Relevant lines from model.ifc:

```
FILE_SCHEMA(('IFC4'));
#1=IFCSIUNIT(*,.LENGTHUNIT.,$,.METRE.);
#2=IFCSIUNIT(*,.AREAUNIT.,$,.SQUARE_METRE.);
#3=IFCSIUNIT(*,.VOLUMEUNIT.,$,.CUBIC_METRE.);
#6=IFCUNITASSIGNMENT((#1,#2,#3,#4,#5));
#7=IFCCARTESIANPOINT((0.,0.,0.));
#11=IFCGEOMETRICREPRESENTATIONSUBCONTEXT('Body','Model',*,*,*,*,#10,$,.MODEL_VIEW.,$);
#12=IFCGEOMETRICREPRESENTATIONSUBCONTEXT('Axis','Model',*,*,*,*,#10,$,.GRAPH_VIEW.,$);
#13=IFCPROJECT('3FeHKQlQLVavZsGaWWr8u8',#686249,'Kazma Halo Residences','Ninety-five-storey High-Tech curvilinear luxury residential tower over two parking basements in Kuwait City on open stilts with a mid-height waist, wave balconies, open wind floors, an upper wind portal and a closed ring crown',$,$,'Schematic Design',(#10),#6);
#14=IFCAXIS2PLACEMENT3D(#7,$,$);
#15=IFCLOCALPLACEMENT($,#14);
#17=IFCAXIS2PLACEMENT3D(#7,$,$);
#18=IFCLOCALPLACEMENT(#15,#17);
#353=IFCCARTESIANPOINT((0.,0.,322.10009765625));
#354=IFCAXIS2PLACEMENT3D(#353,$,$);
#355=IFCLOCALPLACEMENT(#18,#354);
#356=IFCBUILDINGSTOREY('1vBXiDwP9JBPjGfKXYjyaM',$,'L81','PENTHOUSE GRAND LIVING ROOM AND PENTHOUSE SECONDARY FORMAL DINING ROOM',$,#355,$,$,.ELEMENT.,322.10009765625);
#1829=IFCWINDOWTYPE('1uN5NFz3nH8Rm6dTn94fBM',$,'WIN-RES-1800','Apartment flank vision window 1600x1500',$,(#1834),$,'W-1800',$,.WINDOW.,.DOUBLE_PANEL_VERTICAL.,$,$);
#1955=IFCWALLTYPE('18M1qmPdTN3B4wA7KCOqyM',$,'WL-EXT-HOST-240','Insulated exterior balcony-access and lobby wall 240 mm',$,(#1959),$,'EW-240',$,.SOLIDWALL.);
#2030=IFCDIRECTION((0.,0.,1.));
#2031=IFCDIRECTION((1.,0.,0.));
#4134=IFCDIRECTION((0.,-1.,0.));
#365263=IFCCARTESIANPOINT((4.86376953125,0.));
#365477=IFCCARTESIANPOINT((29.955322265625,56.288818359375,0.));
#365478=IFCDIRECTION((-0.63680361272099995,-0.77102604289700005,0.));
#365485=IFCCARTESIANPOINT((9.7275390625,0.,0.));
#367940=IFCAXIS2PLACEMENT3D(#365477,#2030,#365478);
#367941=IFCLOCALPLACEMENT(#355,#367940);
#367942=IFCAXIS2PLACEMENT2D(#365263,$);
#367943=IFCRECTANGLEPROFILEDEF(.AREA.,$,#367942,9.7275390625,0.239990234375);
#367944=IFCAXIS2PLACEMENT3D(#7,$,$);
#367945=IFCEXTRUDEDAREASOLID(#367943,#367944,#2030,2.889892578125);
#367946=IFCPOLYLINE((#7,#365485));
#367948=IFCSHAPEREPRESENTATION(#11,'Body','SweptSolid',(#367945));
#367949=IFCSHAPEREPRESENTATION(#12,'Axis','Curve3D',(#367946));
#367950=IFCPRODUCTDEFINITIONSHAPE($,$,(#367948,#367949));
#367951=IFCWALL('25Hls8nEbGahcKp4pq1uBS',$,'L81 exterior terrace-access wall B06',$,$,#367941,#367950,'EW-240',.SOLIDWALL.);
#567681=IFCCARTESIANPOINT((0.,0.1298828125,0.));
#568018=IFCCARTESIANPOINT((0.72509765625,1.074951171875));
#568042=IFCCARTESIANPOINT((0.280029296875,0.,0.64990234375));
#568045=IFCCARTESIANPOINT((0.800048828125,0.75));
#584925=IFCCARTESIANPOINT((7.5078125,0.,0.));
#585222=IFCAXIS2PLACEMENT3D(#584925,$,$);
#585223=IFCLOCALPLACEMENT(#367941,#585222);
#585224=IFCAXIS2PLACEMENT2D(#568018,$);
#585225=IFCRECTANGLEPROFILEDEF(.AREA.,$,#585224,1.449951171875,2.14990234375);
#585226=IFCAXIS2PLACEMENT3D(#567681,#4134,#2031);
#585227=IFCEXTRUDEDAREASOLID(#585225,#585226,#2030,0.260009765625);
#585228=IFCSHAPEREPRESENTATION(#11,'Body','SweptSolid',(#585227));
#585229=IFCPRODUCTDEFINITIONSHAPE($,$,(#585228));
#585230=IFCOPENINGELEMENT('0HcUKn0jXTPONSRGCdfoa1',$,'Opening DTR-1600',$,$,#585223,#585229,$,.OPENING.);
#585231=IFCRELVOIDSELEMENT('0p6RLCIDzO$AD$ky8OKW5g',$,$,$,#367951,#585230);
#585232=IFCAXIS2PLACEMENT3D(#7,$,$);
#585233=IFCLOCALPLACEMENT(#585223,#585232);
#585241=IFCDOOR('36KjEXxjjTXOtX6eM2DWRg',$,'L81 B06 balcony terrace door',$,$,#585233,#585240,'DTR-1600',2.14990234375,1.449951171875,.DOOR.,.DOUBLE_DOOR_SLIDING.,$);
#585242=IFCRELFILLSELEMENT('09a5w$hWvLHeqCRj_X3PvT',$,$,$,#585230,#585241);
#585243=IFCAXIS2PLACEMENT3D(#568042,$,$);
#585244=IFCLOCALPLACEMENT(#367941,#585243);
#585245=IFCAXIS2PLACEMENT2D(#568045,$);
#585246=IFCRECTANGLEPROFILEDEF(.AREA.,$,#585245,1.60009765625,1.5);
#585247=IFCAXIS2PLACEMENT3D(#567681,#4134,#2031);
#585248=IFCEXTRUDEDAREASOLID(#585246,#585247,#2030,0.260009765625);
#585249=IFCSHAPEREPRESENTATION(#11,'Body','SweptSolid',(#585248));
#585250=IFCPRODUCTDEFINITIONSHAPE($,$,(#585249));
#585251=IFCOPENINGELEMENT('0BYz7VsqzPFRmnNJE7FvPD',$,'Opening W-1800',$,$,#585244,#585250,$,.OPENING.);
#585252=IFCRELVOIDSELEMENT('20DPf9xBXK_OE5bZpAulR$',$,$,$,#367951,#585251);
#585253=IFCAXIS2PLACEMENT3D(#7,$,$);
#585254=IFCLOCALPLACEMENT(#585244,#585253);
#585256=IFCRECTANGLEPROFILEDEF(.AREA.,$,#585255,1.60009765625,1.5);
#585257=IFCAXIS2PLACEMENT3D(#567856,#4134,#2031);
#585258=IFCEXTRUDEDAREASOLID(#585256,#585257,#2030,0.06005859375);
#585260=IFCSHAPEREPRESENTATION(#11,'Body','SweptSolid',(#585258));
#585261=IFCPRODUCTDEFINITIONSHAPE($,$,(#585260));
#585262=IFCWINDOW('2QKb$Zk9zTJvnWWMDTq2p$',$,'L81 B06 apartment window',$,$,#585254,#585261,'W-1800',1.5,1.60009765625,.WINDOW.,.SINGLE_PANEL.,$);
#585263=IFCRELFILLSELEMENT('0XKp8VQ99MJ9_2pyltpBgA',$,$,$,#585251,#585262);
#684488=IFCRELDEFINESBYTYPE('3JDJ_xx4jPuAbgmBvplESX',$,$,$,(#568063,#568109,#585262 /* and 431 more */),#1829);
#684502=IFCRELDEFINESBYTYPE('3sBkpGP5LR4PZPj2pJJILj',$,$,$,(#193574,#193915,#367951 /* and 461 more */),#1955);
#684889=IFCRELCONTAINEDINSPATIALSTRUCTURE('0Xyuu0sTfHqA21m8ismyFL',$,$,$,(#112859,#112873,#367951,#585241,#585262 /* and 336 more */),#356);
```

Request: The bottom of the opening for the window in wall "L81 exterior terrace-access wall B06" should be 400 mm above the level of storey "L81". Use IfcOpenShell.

```python
import numpy as np
import ifcopenshell
import ifcopenshell.api.geometry
import ifcopenshell.geom
import ifcopenshell.util.element
import ifcopenshell.util.placement
import ifcopenshell.util.shape
import ifcopenshell.util.unit

model = ifcopenshell.open("model.ifc")
unit_scale = ifcopenshell.util.unit.calculate_unit_scale(model)

window = model.by_id(585262)
opening = window.FillsVoids[0].RelatingOpeningElement
storey = ifcopenshell.util.element.get_container(window, ifc_class="IfcBuildingStorey")
level = ifcopenshell.util.placement.get_local_placement(storey.ObjectPlacement)[2, 3]

# The opening's origin need not be at the sill, so measure its lowest point.
shape = ifcopenshell.geom.create_shape(ifcopenshell.geom.settings(), opening)
bottom = ifcopenshell.util.shape.get_shape_bottom_elevation(shape, shape.geometry) / unit_scale
dz = level + 0.4 / unit_scale - bottom

shift = np.array([0.0, 0.0, dz])
# The window is placed relative to its opening, so it follows when the opening moves.
matrix = ifcopenshell.util.placement.get_local_placement(opening.ObjectPlacement)
matrix[:3, 3] += shift
ifcopenshell.api.geometry.edit_object_placement(
    model, product=opening, matrix=matrix, is_si=False, should_transform_children=True
)

print(f"moved by {dz * unit_scale:+.3f} m")

model.write("model-out.ifc")
```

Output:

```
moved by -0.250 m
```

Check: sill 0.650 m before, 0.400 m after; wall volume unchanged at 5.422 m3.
